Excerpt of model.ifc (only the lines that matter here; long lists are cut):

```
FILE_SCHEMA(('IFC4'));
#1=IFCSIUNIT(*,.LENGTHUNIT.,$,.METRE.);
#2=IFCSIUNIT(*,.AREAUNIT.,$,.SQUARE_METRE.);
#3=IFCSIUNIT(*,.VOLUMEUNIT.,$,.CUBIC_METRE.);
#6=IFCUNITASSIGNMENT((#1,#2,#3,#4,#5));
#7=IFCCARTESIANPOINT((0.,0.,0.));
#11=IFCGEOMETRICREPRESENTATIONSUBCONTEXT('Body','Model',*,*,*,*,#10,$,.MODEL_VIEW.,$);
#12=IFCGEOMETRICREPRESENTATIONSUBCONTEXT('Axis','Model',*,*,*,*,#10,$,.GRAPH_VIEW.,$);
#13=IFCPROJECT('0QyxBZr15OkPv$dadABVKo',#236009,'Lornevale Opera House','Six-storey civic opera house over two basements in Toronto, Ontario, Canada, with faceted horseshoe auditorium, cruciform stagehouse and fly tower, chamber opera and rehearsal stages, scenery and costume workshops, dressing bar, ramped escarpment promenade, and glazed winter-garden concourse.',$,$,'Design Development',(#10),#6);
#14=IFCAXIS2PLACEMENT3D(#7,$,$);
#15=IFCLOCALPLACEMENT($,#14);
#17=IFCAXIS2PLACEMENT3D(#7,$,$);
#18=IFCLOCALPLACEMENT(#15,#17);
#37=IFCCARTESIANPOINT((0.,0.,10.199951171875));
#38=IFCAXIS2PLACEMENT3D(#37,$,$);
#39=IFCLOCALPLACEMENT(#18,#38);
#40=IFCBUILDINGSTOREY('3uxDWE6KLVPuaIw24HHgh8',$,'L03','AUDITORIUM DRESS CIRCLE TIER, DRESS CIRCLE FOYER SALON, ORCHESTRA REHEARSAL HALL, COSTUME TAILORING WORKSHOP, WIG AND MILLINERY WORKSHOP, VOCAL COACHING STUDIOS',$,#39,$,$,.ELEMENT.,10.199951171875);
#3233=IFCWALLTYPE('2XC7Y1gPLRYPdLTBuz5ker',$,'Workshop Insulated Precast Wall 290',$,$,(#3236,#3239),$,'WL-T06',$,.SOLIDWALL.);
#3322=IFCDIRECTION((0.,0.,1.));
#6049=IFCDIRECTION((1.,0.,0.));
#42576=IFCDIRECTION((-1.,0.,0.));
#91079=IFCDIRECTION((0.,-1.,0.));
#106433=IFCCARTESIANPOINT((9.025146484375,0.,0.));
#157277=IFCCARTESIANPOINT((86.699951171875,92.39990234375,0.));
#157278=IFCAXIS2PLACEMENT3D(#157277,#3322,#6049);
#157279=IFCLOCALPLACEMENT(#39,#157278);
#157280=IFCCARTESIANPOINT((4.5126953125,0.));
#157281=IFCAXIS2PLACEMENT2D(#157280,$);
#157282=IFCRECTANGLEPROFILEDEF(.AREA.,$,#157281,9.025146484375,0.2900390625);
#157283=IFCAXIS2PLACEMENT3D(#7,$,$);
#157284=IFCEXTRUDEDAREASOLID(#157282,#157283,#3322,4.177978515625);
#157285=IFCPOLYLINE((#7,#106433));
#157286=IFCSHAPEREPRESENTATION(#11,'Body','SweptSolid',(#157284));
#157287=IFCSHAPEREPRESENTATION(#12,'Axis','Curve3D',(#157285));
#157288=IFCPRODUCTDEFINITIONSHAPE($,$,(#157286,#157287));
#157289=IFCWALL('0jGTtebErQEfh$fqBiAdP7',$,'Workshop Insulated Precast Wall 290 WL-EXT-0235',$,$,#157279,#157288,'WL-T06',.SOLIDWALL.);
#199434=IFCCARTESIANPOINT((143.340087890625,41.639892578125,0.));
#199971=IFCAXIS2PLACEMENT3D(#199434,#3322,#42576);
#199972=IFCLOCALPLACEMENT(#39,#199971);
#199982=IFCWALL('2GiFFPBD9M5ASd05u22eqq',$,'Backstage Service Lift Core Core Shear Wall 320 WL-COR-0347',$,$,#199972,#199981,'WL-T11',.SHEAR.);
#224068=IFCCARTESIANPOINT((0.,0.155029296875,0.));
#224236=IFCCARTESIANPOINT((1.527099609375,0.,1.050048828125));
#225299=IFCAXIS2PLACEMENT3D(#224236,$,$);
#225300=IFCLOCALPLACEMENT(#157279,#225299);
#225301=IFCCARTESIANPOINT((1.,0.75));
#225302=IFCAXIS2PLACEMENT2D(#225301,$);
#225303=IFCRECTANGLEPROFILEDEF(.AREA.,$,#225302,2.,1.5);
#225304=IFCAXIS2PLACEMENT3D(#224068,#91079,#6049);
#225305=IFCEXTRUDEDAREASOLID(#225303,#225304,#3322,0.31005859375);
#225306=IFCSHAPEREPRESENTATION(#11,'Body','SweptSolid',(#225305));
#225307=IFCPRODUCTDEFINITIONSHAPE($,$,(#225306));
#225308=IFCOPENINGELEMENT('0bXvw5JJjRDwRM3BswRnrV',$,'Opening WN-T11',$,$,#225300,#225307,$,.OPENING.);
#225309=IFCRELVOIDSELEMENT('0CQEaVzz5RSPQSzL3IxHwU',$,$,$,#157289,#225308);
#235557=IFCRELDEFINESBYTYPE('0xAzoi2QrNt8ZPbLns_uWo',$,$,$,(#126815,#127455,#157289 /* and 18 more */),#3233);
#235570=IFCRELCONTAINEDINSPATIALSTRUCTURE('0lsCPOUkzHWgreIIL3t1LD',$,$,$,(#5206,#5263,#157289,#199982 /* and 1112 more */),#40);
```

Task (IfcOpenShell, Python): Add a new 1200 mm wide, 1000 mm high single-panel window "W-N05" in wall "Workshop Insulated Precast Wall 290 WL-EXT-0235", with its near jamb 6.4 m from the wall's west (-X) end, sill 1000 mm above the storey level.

```python
import numpy as np
import ifcopenshell
import ifcopenshell.api.feature
import ifcopenshell.api.geometry
import ifcopenshell.api.root
import ifcopenshell.api.spatial
import ifcopenshell.geom
import ifcopenshell.util.element
import ifcopenshell.util.placement
import ifcopenshell.util.representation
import ifcopenshell.util.shape
import ifcopenshell.util.unit

model = ifcopenshell.open("model.ifc")
unit_scale = ifcopenshell.util.unit.calculate_unit_scale(model)
settings = ifcopenshell.geom.settings()


def volume(element):
    """Net volume in cubic metres, openings subtracted."""
    shape = ifcopenshell.geom.create_shape(settings, element)
    return ifcopenshell.util.shape.get_volume(shape.geometry)


wall = model.by_guid("0jGTtebErQEfh$fqBiAdP7")
storey = ifcopenshell.util.element.get_container(wall, ifc_class="IfcBuildingStorey")
context = ifcopenshell.util.representation.get_context(model, "Model", "Body", "MODEL_VIEW")
before = volume(wall)

width, height, from_end, sill = 1.2, 1, 6.4, 1  # metres

# The wall runs along its own X axis, and the end named is its -X end.
wall_shape = ifcopenshell.geom.create_shape(settings, wall)
x, y, z = ifcopenshell.util.shape.get_vertices(wall_shape.geometry).T
start = x.min() + from_end
face, thickness = float(y.min()), float(y.max() - y.min())
wall_matrix = ifcopenshell.util.placement.get_local_placement(wall.ObjectPlacement)
level = ifcopenshell.util.placement.get_local_placement(storey.ObjectPlacement)[2, 3]


def in_wall(x, y):
    """Placement at x, y metres in the wall's axes, at sill height."""
    matrix = wall_matrix.copy()
    matrix[:, 3] = wall_matrix @ np.array([x / unit_scale, y / unit_scale, 0.0, 1.0])
    matrix[2, 3] = level + sill / unit_scale
    return matrix


# Opening: a box that overshoots both wall faces by 50 mm.
opening = ifcopenshell.api.root.create_entity(model, ifc_class="IfcOpeningElement", predefined_type="OPENING")
box = ifcopenshell.api.geometry.add_wall_representation(
    model, context=context, length=width, height=height, thickness=thickness + 0.1
)
ifcopenshell.api.geometry.assign_representation(model, product=opening, representation=box)
ifcopenshell.api.geometry.edit_object_placement(model, product=opening, matrix=in_wall(start, face - 0.05), is_si=False)
ifcopenshell.api.feature.add_feature(model, feature=opening, element=wall)

window = ifcopenshell.api.root.create_entity(model, ifc_class="IfcWindow", name="W-N05", predefined_type="WINDOW")
window.OverallWidth, window.OverallHeight = width / unit_scale, height / unit_scale
window.PartitioningType = "SINGLE_PANEL"
body = ifcopenshell.api.geometry.add_window_representation(
    model,
    context=context,
    overall_width=window.OverallWidth,
    overall_height=window.OverallHeight,
    partition_type="SINGLE_PANEL",
)
ifcopenshell.api.geometry.assign_representation(model, product=window, representation=body)
ifcopenshell.api.spatial.assign_container(model, products=[window], relating_structure=storey)
ifcopenshell.api.feature.add_filling(model, opening=opening, element=window)

# Centre the window in the wall's thickness.
ifcopenshell.api.geometry.edit_object_placement(model, product=window, matrix=in_wall(start, face), is_si=False)
window_shape = ifcopenshell.geom.create_shape(settings, window)
depth = ifcopenshell.util.shape.get_vertices(window_shape.geometry)[:, 1]
offset = face + thickness / 2 - (depth.min() + depth.max()) / 2
ifcopenshell.api.geometry.edit_object_placement(model, product=window, matrix=in_wall(start, offset), is_si=False)

after = volume(wall)

print(f"wall volume {before:.3f} -> {after:.3f} m3")

model.write("model_edited.ifc")
```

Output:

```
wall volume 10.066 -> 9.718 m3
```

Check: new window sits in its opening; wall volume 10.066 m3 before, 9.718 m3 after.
